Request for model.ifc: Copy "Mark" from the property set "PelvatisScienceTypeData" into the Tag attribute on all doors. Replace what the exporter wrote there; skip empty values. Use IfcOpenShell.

First a look at what the model holds.

```python
import ifcopenshell
import ifcopenshell.util.element

model = ifcopenshell.open("model.ifc")
print(model.schema)
doors = model.by_type("IfcDoor")
print(len(doors), "doors")
for e in doors[:8]:
    source = ifcopenshell.util.element.get_pset(e, "PelvatisScienceTypeData", "Mark")
    target = e.Tag
    print(e.id(), repr(source), repr(target), sep=" | ")
```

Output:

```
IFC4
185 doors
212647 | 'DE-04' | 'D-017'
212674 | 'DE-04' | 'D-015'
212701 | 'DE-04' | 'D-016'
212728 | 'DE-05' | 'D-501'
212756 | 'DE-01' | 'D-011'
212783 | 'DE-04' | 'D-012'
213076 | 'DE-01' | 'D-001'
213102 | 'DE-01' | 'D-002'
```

```python
import ifcopenshell
import ifcopenshell.util.element

model = ifcopenshell.open("model.ifc")

count = 0
for e in model.by_type("IfcDoor"):
    value = ifcopenshell.util.element.get_pset(e, "PelvatisScienceTypeData", "Mark")
    current = e.Tag
    if not value or not value.strip() or current == value:
        continue
    e.Tag = value
    count += 1

print(count, "doors updated")

model.write("model_edited.ifc")
```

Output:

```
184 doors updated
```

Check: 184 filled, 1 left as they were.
